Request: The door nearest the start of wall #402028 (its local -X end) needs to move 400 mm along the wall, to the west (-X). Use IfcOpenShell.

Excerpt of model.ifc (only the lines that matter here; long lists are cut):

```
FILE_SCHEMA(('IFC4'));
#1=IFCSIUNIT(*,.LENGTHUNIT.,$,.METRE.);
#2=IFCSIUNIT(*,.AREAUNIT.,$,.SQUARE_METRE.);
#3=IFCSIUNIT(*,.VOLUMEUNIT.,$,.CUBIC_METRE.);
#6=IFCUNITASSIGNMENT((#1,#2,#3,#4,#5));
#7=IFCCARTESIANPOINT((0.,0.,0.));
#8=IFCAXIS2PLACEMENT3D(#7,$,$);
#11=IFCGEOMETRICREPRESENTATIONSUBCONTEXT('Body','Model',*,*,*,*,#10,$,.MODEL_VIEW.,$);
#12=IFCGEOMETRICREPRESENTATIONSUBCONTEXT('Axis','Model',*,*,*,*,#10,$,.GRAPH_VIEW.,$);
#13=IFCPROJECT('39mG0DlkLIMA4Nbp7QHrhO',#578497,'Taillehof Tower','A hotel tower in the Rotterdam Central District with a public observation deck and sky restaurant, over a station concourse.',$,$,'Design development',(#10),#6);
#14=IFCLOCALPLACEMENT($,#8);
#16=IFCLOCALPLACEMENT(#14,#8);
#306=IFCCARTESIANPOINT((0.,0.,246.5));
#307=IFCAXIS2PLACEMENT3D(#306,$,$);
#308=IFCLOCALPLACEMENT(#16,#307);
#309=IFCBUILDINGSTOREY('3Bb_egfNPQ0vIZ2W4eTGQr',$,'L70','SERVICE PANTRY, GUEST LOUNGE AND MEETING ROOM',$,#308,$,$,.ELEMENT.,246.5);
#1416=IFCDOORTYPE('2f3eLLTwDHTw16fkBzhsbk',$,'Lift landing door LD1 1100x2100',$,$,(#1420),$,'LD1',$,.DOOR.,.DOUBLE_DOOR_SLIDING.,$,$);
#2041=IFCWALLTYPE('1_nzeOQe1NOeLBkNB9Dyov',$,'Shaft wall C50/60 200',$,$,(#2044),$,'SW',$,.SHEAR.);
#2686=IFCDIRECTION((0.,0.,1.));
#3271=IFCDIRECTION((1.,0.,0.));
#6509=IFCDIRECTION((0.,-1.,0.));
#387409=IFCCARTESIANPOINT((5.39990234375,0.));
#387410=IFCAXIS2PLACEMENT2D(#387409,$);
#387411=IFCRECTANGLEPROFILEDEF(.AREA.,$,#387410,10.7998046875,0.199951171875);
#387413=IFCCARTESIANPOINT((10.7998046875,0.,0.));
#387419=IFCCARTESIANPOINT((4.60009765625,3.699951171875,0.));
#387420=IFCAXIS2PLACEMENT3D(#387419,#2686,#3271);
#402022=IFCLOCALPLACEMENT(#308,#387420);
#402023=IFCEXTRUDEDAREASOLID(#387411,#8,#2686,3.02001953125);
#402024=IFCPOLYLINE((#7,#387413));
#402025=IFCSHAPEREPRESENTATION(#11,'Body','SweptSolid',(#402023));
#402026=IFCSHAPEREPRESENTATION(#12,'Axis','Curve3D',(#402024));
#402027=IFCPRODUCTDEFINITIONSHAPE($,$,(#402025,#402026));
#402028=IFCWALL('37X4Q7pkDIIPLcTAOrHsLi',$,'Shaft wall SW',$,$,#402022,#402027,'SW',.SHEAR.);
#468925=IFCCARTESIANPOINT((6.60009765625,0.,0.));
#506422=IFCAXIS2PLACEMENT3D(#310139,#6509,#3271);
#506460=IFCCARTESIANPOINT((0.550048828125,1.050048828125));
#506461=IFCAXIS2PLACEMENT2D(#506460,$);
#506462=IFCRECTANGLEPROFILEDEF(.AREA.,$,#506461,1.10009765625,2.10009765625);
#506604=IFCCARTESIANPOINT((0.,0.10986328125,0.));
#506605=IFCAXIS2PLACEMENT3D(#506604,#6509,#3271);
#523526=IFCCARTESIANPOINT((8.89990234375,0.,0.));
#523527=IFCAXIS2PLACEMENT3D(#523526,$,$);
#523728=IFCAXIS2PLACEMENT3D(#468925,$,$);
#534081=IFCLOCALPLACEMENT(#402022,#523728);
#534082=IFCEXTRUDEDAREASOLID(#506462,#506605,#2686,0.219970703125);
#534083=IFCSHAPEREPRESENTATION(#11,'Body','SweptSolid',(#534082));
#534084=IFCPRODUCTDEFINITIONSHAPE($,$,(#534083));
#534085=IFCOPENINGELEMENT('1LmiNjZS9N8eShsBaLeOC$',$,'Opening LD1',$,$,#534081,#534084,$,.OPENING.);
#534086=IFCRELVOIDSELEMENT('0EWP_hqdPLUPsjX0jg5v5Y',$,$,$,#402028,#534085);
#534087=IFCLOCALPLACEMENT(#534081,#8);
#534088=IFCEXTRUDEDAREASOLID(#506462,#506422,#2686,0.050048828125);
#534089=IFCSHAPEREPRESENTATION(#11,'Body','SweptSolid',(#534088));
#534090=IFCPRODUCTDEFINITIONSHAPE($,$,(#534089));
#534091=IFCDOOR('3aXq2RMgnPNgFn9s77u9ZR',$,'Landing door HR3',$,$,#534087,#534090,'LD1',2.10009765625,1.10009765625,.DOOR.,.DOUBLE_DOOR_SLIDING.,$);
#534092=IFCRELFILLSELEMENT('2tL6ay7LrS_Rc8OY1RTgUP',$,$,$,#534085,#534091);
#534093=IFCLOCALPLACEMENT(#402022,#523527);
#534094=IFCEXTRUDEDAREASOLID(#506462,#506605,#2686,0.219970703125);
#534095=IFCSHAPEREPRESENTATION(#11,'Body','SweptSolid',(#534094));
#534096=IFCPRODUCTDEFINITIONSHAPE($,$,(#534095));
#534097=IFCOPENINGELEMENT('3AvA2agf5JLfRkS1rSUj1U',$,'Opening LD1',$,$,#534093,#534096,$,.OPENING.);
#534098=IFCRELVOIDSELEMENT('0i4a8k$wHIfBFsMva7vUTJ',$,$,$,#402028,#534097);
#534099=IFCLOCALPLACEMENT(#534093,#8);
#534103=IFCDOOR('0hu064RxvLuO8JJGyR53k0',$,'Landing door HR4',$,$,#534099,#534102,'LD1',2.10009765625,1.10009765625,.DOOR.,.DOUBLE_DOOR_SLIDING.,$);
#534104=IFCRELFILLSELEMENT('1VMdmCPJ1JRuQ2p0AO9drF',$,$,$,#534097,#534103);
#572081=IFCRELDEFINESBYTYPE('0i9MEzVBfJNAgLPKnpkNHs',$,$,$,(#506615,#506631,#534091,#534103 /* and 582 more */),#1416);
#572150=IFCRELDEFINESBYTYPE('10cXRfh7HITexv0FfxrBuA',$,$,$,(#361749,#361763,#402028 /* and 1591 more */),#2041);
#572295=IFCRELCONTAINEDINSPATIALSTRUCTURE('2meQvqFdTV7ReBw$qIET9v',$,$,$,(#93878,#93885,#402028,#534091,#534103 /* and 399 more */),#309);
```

```python
import ifcopenshell
import ifcopenshell.api.geometry
import ifcopenshell.util.placement
import ifcopenshell.util.unit

model = ifcopenshell.open("model.ifc")
unit_scale = ifcopenshell.util.unit.calculate_unit_scale(model)

door = model.by_id(534091)
opening = door.FillsVoids[0].RelatingOpeningElement
wall = opening.VoidsElements[0].RelatingBuildingElement

wall_matrix = ifcopenshell.util.placement.get_local_placement(wall.ObjectPlacement)
shift = wall_matrix[:3, 0] * -0.4 / unit_scale
before = ifcopenshell.util.placement.get_local_placement(door.ObjectPlacement)[:3, 3].copy()

# The door is placed relative to its opening, so it follows when the opening moves.
matrix = ifcopenshell.util.placement.get_local_placement(opening.ObjectPlacement)
matrix[:3, 3] += shift
ifcopenshell.api.geometry.edit_object_placement(
    model, product=opening, matrix=matrix, is_si=False, should_transform_children=True
)

after = ifcopenshell.util.placement.get_local_placement(door.ObjectPlacement)[:3, 3]
print("door moved by", (after - before).round(3) + 0.0)

model.write("model-out.ifc")
```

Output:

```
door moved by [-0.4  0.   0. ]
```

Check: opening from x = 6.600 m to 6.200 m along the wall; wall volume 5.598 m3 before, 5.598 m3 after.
